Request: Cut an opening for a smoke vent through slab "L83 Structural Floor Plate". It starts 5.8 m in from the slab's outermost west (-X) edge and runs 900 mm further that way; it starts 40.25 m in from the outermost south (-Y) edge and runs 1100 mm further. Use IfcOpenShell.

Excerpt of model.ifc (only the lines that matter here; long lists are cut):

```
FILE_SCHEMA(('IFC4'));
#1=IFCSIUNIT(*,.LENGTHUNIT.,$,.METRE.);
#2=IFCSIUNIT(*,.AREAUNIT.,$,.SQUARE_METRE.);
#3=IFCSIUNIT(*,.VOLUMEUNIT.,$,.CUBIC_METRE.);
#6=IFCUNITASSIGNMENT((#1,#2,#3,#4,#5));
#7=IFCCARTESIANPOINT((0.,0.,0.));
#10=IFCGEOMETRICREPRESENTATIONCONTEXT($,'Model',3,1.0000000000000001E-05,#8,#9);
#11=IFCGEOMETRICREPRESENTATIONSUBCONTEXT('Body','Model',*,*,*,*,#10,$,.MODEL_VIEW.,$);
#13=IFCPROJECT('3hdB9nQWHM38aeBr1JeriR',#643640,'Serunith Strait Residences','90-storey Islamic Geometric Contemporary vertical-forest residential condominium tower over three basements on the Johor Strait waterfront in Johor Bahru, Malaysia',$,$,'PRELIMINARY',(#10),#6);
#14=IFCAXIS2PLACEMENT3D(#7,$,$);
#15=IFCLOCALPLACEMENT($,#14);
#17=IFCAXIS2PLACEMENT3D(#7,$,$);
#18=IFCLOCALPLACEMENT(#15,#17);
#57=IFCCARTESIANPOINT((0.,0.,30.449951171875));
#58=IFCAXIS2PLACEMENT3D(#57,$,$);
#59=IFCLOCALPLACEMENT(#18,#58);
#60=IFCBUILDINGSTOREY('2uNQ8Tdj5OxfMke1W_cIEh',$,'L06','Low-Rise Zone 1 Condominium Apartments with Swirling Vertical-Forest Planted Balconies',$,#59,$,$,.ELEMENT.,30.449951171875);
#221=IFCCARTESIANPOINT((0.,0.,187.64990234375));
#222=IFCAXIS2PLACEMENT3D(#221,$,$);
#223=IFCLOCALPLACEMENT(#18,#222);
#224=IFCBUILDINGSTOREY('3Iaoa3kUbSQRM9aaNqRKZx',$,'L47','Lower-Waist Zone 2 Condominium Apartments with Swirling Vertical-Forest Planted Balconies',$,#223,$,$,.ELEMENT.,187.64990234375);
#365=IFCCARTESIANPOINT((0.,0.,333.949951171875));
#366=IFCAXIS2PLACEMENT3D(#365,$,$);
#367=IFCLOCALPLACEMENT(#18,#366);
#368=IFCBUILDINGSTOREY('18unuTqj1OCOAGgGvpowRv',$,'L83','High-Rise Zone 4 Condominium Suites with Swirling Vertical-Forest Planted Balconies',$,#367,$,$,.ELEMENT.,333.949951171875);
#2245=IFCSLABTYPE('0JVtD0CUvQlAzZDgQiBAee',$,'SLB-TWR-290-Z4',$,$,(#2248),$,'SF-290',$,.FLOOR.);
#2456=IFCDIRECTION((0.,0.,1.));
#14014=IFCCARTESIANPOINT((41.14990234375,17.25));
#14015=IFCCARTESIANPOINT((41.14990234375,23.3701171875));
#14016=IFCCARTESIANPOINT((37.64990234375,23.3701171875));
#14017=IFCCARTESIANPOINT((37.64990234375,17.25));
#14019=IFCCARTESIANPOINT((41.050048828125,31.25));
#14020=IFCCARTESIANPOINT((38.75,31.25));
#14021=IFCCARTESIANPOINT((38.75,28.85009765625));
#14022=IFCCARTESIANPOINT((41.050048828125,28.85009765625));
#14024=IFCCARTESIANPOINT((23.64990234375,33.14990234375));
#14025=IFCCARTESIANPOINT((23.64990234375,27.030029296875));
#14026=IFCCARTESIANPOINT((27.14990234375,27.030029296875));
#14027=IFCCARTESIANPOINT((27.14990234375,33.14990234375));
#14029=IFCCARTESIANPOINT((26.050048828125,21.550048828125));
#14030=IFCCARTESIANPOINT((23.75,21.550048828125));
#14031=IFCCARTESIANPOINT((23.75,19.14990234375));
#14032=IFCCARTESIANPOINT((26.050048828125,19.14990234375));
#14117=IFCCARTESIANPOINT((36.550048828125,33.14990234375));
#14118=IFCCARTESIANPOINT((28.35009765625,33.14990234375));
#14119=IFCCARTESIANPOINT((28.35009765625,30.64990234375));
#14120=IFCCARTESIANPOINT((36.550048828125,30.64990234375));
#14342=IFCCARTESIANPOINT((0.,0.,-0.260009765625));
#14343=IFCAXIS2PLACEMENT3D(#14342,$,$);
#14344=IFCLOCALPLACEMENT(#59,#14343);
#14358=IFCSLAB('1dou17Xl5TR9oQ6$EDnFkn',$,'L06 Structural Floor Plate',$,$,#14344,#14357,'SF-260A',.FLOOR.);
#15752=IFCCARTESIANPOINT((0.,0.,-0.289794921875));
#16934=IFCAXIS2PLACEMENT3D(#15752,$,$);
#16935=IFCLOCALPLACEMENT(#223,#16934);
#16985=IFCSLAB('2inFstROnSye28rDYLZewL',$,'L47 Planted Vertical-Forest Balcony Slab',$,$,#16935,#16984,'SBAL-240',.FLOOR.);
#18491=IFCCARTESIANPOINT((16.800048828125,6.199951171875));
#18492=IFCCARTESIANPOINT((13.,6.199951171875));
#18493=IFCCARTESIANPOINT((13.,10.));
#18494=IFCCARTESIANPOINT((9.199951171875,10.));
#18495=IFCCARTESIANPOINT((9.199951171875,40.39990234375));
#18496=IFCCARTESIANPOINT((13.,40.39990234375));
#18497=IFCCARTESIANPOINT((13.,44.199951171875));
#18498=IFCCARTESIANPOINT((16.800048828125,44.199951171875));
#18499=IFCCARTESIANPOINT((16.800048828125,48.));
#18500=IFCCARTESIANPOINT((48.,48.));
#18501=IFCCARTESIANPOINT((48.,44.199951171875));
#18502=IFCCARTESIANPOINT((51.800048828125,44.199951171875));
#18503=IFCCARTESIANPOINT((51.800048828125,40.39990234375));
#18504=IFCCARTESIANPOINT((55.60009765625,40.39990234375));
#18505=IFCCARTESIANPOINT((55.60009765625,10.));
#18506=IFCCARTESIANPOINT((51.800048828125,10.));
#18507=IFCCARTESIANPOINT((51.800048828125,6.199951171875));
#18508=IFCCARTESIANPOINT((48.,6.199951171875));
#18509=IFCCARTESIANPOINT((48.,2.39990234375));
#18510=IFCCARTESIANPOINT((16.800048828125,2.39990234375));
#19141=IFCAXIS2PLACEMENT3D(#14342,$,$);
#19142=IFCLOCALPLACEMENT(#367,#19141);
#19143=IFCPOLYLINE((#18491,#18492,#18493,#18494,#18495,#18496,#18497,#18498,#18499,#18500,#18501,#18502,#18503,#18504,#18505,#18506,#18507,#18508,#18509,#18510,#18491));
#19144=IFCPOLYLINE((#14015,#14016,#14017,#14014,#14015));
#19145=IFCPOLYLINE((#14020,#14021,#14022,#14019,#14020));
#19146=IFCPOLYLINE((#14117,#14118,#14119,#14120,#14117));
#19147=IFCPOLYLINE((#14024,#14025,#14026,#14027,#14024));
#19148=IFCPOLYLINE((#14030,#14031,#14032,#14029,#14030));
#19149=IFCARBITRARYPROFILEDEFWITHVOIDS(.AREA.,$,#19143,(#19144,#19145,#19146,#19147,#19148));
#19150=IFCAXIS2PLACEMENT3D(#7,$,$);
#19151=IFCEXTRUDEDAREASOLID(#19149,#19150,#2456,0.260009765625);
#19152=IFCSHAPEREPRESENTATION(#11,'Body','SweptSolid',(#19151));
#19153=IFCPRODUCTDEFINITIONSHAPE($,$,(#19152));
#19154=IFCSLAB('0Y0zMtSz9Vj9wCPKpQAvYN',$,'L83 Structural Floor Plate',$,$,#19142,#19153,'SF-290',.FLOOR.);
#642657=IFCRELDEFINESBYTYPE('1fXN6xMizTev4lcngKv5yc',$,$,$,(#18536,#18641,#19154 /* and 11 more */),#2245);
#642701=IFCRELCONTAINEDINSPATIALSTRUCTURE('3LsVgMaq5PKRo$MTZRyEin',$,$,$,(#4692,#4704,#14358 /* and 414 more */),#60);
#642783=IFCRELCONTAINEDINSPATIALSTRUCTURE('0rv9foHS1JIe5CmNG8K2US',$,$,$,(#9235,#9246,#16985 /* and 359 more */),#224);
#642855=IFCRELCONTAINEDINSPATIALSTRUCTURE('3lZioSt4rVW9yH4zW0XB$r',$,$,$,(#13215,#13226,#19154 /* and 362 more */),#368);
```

```python
import numpy as np
import ifcopenshell
import ifcopenshell.api.feature
import ifcopenshell.api.geometry
import ifcopenshell.api.root
import ifcopenshell.geom
import ifcopenshell.util.placement
import ifcopenshell.util.representation
import ifcopenshell.util.shape
import ifcopenshell.util.unit

model = ifcopenshell.open("model.ifc")
unit_scale = ifcopenshell.util.unit.calculate_unit_scale(model)
settings = ifcopenshell.geom.settings()


def volume(element):
    """Net volume in cubic metres, openings subtracted."""
    shape = ifcopenshell.geom.create_shape(settings, element)
    return ifcopenshell.util.shape.get_volume(shape.geometry)


slab = model.by_guid("0Y0zMtSz9Vj9wCPKpQAvYN")
before = volume(slab)

# Extent in the slab's own axes, in metres. The edges named are its -X and -Y sides.
slab_shape = ifcopenshell.geom.create_shape(settings, slab)
vertices = ifcopenshell.util.shape.get_vertices(slab_shape.geometry)
x_min, y_min, bottom = vertices.min(axis=0)
top = vertices[:, 2].max()

opening = ifcopenshell.api.root.create_entity(model, ifc_class="IfcOpeningElement", name="Smoke vent opening", predefined_type="OPENING")
context = ifcopenshell.util.representation.get_context(model, "Model", "Body", "MODEL_VIEW")
width, depth = 0.9, 1.1
outline = [(0.0, 0.0), (width, 0.0), (width, depth), (0.0, depth), (0.0, 0.0)]
# Overshoot both faces by 50 mm so the cut is clean.
shape = ifcopenshell.api.geometry.add_slab_representation(
    model, context=context, depth=top - bottom + 0.1, polyline=outline
)
ifcopenshell.api.geometry.assign_representation(model, product=opening, representation=shape)

matrix = ifcopenshell.util.placement.get_local_placement(slab.ObjectPlacement)
matrix[:, 3] = matrix @ np.append(np.array([x_min + 5.8, y_min + 40.25, bottom - 0.05]) / unit_scale, 1.0)
ifcopenshell.api.geometry.edit_object_placement(model, product=opening, matrix=matrix, is_si=False)
ifcopenshell.api.feature.add_feature(model, feature=opening, element=slab)

after = volume(slab)

print(f"slab volume {before:.3f} -> {after:.3f} m3")

model.write("model_v2.ifc")
```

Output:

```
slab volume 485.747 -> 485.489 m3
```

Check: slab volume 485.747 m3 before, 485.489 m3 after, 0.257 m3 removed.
